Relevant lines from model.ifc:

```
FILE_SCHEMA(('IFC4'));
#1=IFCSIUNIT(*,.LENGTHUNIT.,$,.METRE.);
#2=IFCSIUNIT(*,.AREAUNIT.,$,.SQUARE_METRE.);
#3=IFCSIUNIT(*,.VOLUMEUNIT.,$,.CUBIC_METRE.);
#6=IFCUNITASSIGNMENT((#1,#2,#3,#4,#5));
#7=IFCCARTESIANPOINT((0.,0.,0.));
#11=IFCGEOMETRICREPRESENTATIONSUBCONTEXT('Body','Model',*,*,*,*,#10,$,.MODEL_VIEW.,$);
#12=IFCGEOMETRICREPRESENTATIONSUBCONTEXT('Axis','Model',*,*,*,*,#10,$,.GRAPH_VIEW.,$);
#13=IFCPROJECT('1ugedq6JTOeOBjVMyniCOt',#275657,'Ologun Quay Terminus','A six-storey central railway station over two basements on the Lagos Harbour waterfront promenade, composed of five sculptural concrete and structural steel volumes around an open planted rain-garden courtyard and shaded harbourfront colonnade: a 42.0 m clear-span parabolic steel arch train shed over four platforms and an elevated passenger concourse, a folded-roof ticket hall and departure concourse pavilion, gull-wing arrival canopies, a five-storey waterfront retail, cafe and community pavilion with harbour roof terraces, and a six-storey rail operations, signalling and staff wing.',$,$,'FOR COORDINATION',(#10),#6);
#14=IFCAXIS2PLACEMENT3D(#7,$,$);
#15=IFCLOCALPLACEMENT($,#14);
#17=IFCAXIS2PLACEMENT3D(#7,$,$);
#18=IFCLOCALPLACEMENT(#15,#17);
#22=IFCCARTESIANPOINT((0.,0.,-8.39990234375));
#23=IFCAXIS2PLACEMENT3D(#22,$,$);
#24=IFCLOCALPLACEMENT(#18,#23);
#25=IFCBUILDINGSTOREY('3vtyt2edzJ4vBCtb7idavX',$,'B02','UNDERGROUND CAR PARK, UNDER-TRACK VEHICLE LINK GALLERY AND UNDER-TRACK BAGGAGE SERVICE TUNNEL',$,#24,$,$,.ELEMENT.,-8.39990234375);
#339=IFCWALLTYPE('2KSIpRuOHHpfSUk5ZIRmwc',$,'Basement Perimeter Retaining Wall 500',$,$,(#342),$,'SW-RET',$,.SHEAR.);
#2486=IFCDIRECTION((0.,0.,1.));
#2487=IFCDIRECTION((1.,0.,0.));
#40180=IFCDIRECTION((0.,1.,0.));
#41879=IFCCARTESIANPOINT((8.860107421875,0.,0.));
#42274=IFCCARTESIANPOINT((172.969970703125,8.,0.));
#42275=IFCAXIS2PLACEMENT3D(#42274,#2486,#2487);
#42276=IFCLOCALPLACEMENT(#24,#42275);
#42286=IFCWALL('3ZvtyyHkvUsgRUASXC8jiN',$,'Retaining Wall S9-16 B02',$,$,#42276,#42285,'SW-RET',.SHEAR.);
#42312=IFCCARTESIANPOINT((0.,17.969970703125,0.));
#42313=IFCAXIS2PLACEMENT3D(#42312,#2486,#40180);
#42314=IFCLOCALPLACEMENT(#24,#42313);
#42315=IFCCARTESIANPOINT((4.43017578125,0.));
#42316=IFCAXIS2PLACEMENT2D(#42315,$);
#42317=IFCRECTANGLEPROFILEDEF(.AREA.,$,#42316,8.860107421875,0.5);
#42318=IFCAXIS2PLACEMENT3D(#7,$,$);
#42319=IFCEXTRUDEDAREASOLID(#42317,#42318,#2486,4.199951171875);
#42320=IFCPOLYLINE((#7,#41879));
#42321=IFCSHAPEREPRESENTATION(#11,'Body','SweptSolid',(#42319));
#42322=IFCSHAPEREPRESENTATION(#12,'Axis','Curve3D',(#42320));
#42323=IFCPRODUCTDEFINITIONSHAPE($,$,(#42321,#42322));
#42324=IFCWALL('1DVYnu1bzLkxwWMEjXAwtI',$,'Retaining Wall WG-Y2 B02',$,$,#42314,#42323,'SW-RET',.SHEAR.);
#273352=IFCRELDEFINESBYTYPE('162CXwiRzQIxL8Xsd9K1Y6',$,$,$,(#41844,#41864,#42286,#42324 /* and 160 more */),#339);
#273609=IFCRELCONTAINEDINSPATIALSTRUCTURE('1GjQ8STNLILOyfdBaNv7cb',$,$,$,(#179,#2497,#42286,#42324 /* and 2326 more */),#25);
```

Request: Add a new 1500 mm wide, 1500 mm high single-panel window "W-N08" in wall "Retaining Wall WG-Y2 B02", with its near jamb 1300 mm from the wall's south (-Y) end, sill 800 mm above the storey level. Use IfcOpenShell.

```python
import numpy as np
import ifcopenshell
import ifcopenshell.api.feature
import ifcopenshell.api.geometry
import ifcopenshell.api.root
import ifcopenshell.api.spatial
import ifcopenshell.geom
import ifcopenshell.util.element
import ifcopenshell.util.placement
import ifcopenshell.util.representation
import ifcopenshell.util.shape
import ifcopenshell.util.unit

model = ifcopenshell.open("model.ifc")
unit_scale = ifcopenshell.util.unit.calculate_unit_scale(model)
settings = ifcopenshell.geom.settings()


def volume(element):
    """Net volume in cubic metres, openings subtracted."""
    shape = ifcopenshell.geom.create_shape(settings, element)
    return ifcopenshell.util.shape.get_volume(shape.geometry)


wall = model.by_guid("1DVYnu1bzLkxwWMEjXAwtI")
storey = ifcopenshell.util.element.get_container(wall, ifc_class="IfcBuildingStorey")
context = ifcopenshell.util.representation.get_context(model, "Model", "Body", "MODEL_VIEW")
before = volume(wall)

width, height, from_end, sill = 1.5, 1.5, 1.3, 0.8  # metres

# The wall runs along its own X axis, and the end named is its -X end.
wall_shape = ifcopenshell.geom.create_shape(settings, wall)
x, y, z = ifcopenshell.util.shape.get_vertices(wall_shape.geometry).T
start = x.min() + from_end
face, thickness = float(y.min()), float(y.max() - y.min())
wall_matrix = ifcopenshell.util.placement.get_local_placement(wall.ObjectPlacement)
level = ifcopenshell.util.placement.get_local_placement(storey.ObjectPlacement)[2, 3]


def in_wall(x, y):
    """Placement at x, y metres in the wall's axes, at sill height."""
    matrix = wall_matrix.copy()
    matrix[:, 3] = wall_matrix @ np.array([x / unit_scale, y / unit_scale, 0.0, 1.0])
    matrix[2, 3] = level + sill / unit_scale
    return matrix


# Opening: a box that overshoots both wall faces by 50 mm.
opening = ifcopenshell.api.root.create_entity(model, ifc_class="IfcOpeningElement", predefined_type="OPENING")
box = ifcopenshell.api.geometry.add_wall_representation(
    model, context=context, length=width, height=height, thickness=thickness + 0.1
)
ifcopenshell.api.geometry.assign_representation(model, product=opening, representation=box)
ifcopenshell.api.geometry.edit_object_placement(model, product=opening, matrix=in_wall(start, face - 0.05), is_si=False)
ifcopenshell.api.feature.add_feature(model, feature=opening, element=wall)

window = ifcopenshell.api.root.create_entity(model, ifc_class="IfcWindow", name="W-N08", predefined_type="WINDOW")
window.OverallWidth, window.OverallHeight = width / unit_scale, height / unit_scale
window.PartitioningType = "SINGLE_PANEL"
body = ifcopenshell.api.geometry.add_window_representation(
    model,
    context=context,
    overall_width=window.OverallWidth,
    overall_height=window.OverallHeight,
    partition_type="SINGLE_PANEL",
)
ifcopenshell.api.geometry.assign_representation(model, product=window, representation=body)
ifcopenshell.api.spatial.assign_container(model, products=[window], relating_structure=storey)
ifcopenshell.api.feature.add_filling(model, opening=opening, element=window)

# Centre the window in the wall's thickness.
ifcopenshell.api.geometry.edit_object_placement(model, product=window, matrix=in_wall(start, face), is_si=False)
window_shape = ifcopenshell.geom.create_shape(settings, window)
depth = ifcopenshell.util.shape.get_vertices(window_shape.geometry)[:, 1]
offset = face + thickness / 2 - (depth.min() + depth.max()) / 2
ifcopenshell.api.geometry.edit_object_placement(model, product=window, matrix=in_wall(start, offset), is_si=False)

after = volume(wall)

print(f"wall volume {before:.3f} -> {after:.3f} m3")

model.write("model_edited.ifc")
```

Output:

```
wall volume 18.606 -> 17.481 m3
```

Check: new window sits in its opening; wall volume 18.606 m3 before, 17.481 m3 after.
